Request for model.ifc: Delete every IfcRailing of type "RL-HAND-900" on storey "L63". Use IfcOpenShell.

First a look at what the model holds.

```python
import ifcopenshell
import ifcopenshell.util.element

model = ifcopenshell.open("model.ifc")
print(model.schema)
storey = next(s for s in model.by_type("IfcBuildingStorey") if s.Name == "L63")
railings = [e for e in ifcopenshell.util.element.get_decomposition(storey) if e.is_a("IfcRailing")]
seen = {}
for e in railings:
    element_type = ifcopenshell.util.element.get_type(e)
    name = element_type.Name if element_type not in (None, e) else None
    seen[name] = seen.get(name, 0) + 1
for name, count in sorted(seen.items(), key=str):
    print(count, "x", name)
```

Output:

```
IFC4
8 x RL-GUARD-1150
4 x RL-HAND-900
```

```python
import ifcopenshell
import ifcopenshell.api.root
import ifcopenshell.util.element

model = ifcopenshell.open("model.ifc")

storey = next(s for s in model.by_type("IfcBuildingStorey") if s.Name == "L63")
railings = [e for e in ifcopenshell.util.element.get_decomposition(storey) if e.is_a("IfcRailing")]
targets = [e for e in railings if (t := ifcopenshell.util.element.get_type(e)) not in (None, e) and t.Name == "RL-HAND-900"]

for e in targets:
    ifcopenshell.api.root.remove_product(model, product=e)
print(len(targets), "removed")

model.write("model-out.ifc")
```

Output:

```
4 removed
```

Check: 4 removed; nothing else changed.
